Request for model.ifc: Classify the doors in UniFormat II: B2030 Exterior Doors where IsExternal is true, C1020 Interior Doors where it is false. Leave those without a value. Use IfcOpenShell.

First a look at what the model holds.

```python
import ifcopenshell
import ifcopenshell.util.element

model = ifcopenshell.open("model.ifc")
print(model.schema)
print("classifications:", [c.Name for c in model.by_type("IfcClassification")])
values = [ifcopenshell.util.element.get_pset(e, "Pset_DoorCommon", "IsExternal") for e in model.by_type("IfcDoor")]
for value in (True, False, None):
    print("IsExternal", value, values.count(value))
```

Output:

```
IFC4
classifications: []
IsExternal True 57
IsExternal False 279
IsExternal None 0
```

```python
import ifcopenshell
import ifcopenshell.api.classification
import ifcopenshell.util.element

model = ifcopenshell.open("model.ifc")

system = ifcopenshell.api.classification.add_classification(model, classification="UniFormat II")

doors = model.by_type("IfcDoor")
external = {e: ifcopenshell.util.element.get_pset(e, "Pset_DoorCommon", "IsExternal") for e in doors}
for flag, code, name in ((True, "B2030", "Exterior Doors"), (False, "C1020", "Interior Doors")):
    products = [e for e in doors if external[e] is flag]
    ifcopenshell.api.classification.add_reference(
        model, products=products, classification=system, identification=code, name=name
    )
    print(code, len(products))

model.write("model_v2.ifc")
```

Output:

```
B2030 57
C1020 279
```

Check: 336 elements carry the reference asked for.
